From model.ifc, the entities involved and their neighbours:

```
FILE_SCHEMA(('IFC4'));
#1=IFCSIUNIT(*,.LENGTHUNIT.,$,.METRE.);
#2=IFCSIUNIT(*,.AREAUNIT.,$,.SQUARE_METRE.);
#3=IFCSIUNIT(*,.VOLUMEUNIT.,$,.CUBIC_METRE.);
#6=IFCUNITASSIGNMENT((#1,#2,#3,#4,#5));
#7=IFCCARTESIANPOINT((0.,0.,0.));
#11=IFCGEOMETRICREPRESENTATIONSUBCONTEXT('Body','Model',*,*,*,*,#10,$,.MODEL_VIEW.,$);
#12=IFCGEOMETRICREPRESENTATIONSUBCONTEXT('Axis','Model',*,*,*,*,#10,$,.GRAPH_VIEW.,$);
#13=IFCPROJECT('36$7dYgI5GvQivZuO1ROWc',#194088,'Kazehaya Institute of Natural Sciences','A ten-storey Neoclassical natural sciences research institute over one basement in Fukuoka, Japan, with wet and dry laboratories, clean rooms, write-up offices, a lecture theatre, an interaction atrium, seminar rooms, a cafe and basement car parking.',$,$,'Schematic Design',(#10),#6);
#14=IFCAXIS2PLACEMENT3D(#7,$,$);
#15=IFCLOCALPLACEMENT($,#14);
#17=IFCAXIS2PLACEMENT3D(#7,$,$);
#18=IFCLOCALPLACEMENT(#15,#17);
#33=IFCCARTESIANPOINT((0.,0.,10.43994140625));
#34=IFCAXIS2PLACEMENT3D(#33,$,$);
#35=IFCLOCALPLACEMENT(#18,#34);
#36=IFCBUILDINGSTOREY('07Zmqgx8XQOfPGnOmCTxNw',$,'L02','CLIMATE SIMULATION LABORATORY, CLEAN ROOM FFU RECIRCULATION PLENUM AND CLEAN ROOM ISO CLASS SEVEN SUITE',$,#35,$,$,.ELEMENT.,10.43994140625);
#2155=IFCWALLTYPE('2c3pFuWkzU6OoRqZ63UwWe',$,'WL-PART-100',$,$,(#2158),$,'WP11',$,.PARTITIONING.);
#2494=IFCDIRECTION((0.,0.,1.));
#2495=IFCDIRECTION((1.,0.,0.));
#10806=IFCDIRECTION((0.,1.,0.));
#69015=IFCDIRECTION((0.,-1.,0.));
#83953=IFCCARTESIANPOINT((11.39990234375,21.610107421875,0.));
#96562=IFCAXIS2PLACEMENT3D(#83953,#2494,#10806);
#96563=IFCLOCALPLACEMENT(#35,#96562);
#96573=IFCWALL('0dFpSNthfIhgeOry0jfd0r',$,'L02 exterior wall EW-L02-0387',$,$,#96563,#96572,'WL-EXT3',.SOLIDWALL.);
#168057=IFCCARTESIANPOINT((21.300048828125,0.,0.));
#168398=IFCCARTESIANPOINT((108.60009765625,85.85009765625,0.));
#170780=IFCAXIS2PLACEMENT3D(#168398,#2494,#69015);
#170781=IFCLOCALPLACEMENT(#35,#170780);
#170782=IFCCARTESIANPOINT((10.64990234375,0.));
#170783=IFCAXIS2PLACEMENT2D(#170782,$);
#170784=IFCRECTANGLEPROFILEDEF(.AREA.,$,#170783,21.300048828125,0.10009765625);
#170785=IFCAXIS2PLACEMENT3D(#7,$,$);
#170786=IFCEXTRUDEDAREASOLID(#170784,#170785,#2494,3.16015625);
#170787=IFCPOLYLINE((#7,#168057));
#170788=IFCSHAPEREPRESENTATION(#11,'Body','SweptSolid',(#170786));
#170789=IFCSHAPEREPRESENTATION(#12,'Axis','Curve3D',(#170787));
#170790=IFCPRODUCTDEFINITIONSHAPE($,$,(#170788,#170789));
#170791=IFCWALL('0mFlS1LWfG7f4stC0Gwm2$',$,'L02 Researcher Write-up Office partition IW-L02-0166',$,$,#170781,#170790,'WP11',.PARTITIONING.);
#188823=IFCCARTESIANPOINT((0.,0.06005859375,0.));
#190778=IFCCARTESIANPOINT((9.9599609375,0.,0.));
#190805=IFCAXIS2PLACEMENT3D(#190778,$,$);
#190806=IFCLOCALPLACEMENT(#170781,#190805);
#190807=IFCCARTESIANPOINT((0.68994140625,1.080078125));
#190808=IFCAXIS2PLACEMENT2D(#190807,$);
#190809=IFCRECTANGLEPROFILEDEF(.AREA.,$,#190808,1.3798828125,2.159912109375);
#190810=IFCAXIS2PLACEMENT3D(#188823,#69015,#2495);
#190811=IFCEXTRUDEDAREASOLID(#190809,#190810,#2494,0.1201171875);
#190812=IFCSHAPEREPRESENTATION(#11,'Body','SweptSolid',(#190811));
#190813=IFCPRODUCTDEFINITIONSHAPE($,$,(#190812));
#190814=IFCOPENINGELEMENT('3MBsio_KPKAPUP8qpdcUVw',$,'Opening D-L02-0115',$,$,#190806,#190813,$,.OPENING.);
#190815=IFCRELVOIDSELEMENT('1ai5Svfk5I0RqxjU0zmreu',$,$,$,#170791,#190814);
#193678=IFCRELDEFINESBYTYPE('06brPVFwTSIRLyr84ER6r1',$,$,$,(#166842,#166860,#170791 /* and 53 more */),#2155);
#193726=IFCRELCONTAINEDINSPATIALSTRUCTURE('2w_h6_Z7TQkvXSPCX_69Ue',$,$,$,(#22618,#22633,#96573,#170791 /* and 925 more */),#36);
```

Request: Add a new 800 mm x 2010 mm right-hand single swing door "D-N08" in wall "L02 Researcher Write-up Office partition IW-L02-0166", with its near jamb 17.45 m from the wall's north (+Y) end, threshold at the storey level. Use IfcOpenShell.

```python
import numpy as np
import ifcopenshell
import ifcopenshell.api.feature
import ifcopenshell.api.geometry
import ifcopenshell.api.root
import ifcopenshell.api.spatial
import ifcopenshell.geom
import ifcopenshell.util.element
import ifcopenshell.util.placement
import ifcopenshell.util.representation
import ifcopenshell.util.shape
import ifcopenshell.util.unit

model = ifcopenshell.open("model.ifc")
unit_scale = ifcopenshell.util.unit.calculate_unit_scale(model)
settings = ifcopenshell.geom.settings()


def volume(element):
    """Net volume in cubic metres, openings subtracted."""
    shape = ifcopenshell.geom.create_shape(settings, element)
    return ifcopenshell.util.shape.get_volume(shape.geometry)


wall = model.by_id(170791)
storey = ifcopenshell.util.element.get_container(wall, ifc_class="IfcBuildingStorey")
context = ifcopenshell.util.representation.get_context(model, "Model", "Body", "MODEL_VIEW")
before = volume(wall)

width, height, from_end, sill = 0.8, 2.01, 17.45, 0.0  # metres

# The wall runs along its own X axis, and the end named is its -X end.
wall_shape = ifcopenshell.geom.create_shape(settings, wall)
x, y, z = ifcopenshell.util.shape.get_vertices(wall_shape.geometry).T
start = x.min() + from_end
face, thickness = float(y.min()), float(y.max() - y.min())
wall_matrix = ifcopenshell.util.placement.get_local_placement(wall.ObjectPlacement)
level = ifcopenshell.util.placement.get_local_placement(storey.ObjectPlacement)[2, 3]


def in_wall(x, y):
    """Placement at x, y metres in the wall's axes, at sill height."""
    matrix = wall_matrix.copy()
    matrix[:, 3] = wall_matrix @ np.array([x / unit_scale, y / unit_scale, 0.0, 1.0])
    matrix[2, 3] = level + sill / unit_scale
    return matrix


# Opening: a box that overshoots both wall faces by 50 mm.
opening = ifcopenshell.api.root.create_entity(model, ifc_class="IfcOpeningElement", predefined_type="OPENING")
box = ifcopenshell.api.geometry.add_wall_representation(
    model, context=context, length=width, height=height, thickness=thickness + 0.1
)
ifcopenshell.api.geometry.assign_representation(model, product=opening, representation=box)
ifcopenshell.api.geometry.edit_object_placement(model, product=opening, matrix=in_wall(start, face - 0.05), is_si=False)
ifcopenshell.api.feature.add_feature(model, feature=opening, element=wall)

door = ifcopenshell.api.root.create_entity(model, ifc_class="IfcDoor", name="D-N08", predefined_type="DOOR")
door.OverallWidth, door.OverallHeight = width / unit_scale, height / unit_scale
door.OperationType = "SINGLE_SWING_RIGHT"
body = ifcopenshell.api.geometry.add_door_representation(
    model,
    context=context,
    overall_width=door.OverallWidth,
    overall_height=door.OverallHeight,
    operation_type="SINGLE_SWING_RIGHT",
    lining_properties={"LiningDepth": thickness / unit_scale, "ThresholdDepth": thickness / unit_scale},
)
ifcopenshell.api.geometry.assign_representation(model, product=door, representation=body)
ifcopenshell.api.spatial.assign_container(model, products=[door], relating_structure=storey)
ifcopenshell.api.feature.add_filling(model, opening=opening, element=door)

# The lining spans the wall, so the door starts at the wall face.
ifcopenshell.api.geometry.edit_object_placement(model, product=door, matrix=in_wall(start, face), is_si=False)

after = volume(wall)

print(f"wall volume {before:.3f} -> {after:.3f} m3")

model.write("model_edited.ifc")
```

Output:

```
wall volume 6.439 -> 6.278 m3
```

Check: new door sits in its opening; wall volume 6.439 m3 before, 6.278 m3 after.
